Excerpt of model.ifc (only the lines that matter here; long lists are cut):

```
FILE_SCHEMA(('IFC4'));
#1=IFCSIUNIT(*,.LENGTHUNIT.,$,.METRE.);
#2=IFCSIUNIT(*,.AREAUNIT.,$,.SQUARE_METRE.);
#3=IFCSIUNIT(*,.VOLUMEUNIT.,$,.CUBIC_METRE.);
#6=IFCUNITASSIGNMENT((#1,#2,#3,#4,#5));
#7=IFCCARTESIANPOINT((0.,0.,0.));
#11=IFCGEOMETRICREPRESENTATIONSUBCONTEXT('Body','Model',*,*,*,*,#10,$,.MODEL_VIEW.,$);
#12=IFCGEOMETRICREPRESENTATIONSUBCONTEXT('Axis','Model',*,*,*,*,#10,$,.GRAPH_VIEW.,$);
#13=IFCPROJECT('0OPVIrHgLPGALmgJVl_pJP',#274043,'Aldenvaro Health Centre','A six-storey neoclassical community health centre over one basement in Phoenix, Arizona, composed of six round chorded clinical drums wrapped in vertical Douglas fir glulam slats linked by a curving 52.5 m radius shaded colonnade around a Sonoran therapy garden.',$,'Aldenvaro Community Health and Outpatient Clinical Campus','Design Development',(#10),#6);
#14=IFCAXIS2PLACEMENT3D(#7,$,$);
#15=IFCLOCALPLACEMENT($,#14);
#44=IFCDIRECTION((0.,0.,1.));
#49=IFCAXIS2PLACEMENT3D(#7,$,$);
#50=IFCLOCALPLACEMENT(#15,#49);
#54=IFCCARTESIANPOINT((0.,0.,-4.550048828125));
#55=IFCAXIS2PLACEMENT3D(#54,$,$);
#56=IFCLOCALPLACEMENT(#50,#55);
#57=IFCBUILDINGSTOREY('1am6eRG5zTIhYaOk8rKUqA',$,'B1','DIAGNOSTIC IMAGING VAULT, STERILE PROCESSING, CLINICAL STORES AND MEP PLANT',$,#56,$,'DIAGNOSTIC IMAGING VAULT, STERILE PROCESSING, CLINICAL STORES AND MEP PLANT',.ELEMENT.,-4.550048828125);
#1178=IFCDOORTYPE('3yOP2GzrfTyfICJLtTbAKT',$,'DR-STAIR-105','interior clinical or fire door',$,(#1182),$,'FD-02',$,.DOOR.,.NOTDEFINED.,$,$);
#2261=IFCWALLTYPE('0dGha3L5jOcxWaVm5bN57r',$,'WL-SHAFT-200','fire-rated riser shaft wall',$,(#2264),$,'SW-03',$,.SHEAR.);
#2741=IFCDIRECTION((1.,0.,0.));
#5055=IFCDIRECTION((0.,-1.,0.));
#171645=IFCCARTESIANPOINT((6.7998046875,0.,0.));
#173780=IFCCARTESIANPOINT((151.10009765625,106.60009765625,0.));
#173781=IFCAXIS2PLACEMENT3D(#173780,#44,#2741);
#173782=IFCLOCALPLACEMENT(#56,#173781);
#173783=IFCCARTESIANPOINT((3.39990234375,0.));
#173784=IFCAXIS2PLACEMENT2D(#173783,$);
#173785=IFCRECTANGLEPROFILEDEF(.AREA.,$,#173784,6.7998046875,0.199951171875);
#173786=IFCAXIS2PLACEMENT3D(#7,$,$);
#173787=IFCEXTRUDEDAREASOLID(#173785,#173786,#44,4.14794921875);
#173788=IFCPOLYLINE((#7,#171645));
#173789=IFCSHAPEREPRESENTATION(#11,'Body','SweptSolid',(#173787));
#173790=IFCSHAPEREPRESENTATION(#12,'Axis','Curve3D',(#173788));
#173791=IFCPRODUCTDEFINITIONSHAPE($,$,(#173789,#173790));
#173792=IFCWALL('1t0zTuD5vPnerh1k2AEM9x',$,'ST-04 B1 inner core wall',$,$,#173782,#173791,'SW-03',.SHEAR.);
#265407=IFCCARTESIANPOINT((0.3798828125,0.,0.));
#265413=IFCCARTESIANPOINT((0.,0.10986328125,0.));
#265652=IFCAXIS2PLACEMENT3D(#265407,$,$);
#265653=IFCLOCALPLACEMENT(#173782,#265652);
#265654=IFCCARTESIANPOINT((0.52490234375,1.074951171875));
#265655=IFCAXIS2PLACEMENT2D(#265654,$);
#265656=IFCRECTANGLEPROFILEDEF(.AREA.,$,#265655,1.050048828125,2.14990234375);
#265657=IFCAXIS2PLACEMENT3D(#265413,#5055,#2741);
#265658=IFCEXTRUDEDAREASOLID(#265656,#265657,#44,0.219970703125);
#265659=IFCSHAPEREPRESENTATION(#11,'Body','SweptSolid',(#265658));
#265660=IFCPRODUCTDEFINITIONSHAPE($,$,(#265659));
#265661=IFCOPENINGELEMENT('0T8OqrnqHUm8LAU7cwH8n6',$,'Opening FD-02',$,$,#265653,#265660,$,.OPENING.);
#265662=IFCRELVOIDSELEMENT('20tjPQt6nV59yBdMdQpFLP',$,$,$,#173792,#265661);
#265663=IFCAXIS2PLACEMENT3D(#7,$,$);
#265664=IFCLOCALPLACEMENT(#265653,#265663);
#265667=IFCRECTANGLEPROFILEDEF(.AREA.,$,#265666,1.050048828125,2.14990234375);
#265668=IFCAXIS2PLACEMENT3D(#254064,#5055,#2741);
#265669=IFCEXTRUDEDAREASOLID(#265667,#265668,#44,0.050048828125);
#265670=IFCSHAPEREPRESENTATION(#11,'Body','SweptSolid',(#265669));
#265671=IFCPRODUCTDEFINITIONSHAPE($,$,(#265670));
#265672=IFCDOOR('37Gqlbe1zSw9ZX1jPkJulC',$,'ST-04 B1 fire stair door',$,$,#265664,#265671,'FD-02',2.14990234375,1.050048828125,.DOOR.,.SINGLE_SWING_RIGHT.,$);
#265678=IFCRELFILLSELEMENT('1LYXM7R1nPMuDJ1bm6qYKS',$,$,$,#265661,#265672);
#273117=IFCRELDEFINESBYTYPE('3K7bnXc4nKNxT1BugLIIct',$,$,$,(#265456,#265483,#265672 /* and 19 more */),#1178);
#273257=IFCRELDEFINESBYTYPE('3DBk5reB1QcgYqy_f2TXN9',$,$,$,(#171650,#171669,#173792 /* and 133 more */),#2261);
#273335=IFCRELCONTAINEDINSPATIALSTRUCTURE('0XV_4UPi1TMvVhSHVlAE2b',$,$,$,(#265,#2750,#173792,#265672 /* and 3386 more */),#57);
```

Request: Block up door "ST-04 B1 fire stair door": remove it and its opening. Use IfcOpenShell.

```python
import ifcopenshell
import ifcopenshell.api.feature
import ifcopenshell.api.root
import ifcopenshell.geom
import ifcopenshell.util.shape

model = ifcopenshell.open("model.ifc")
settings = ifcopenshell.geom.settings()


def volume(element):
    """Net volume in cubic metres, openings subtracted."""
    shape = ifcopenshell.geom.create_shape(settings, element)
    return ifcopenshell.util.shape.get_volume(shape.geometry)


door = model.by_id(265672)
opening = door.FillsVoids[0].RelatingOpeningElement
wall = opening.VoidsElements[0].RelatingBuildingElement
before = volume(wall)

ifcopenshell.api.root.remove_product(model, product=door)
ifcopenshell.api.feature.remove_feature(model, feature=opening)

after = volume(wall)

print(f"wall volume {before:.3f} -> {after:.3f} m3")

model.write("model_updated.ifc")
```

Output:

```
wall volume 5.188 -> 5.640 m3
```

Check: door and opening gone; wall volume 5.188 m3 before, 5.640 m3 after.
